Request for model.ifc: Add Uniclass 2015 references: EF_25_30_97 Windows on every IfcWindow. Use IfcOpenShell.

First a look at what the model holds.

```python
import ifcopenshell

model = ifcopenshell.open("model.ifc")
print(model.schema)
print("classifications:", [c.Name for c in model.by_type("IfcClassification")])
for ifc_class in ("IfcDoor", "IfcRoof", "IfcStair", "IfcWall", "IfcWindow"):
    print(ifc_class, len(model.by_type(ifc_class)))
```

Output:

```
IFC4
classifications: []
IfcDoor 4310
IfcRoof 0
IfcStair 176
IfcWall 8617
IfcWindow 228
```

```python
import ifcopenshell
import ifcopenshell.api.classification

model = ifcopenshell.open("model.ifc")

system = ifcopenshell.api.classification.add_classification(model, classification="Uniclass 2015")

codes = {
    "IfcWindow": ("EF_25_30_97", "Windows"),
}
for ifc_class, (code, name) in codes.items():
    products = model.by_type(ifc_class)
    ifcopenshell.api.classification.add_reference(
        model, products=products, classification=system, identification=code, name=name
    )
    print(code, len(products))

model.write("model-out.ifc")
```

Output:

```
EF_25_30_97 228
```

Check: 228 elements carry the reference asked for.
